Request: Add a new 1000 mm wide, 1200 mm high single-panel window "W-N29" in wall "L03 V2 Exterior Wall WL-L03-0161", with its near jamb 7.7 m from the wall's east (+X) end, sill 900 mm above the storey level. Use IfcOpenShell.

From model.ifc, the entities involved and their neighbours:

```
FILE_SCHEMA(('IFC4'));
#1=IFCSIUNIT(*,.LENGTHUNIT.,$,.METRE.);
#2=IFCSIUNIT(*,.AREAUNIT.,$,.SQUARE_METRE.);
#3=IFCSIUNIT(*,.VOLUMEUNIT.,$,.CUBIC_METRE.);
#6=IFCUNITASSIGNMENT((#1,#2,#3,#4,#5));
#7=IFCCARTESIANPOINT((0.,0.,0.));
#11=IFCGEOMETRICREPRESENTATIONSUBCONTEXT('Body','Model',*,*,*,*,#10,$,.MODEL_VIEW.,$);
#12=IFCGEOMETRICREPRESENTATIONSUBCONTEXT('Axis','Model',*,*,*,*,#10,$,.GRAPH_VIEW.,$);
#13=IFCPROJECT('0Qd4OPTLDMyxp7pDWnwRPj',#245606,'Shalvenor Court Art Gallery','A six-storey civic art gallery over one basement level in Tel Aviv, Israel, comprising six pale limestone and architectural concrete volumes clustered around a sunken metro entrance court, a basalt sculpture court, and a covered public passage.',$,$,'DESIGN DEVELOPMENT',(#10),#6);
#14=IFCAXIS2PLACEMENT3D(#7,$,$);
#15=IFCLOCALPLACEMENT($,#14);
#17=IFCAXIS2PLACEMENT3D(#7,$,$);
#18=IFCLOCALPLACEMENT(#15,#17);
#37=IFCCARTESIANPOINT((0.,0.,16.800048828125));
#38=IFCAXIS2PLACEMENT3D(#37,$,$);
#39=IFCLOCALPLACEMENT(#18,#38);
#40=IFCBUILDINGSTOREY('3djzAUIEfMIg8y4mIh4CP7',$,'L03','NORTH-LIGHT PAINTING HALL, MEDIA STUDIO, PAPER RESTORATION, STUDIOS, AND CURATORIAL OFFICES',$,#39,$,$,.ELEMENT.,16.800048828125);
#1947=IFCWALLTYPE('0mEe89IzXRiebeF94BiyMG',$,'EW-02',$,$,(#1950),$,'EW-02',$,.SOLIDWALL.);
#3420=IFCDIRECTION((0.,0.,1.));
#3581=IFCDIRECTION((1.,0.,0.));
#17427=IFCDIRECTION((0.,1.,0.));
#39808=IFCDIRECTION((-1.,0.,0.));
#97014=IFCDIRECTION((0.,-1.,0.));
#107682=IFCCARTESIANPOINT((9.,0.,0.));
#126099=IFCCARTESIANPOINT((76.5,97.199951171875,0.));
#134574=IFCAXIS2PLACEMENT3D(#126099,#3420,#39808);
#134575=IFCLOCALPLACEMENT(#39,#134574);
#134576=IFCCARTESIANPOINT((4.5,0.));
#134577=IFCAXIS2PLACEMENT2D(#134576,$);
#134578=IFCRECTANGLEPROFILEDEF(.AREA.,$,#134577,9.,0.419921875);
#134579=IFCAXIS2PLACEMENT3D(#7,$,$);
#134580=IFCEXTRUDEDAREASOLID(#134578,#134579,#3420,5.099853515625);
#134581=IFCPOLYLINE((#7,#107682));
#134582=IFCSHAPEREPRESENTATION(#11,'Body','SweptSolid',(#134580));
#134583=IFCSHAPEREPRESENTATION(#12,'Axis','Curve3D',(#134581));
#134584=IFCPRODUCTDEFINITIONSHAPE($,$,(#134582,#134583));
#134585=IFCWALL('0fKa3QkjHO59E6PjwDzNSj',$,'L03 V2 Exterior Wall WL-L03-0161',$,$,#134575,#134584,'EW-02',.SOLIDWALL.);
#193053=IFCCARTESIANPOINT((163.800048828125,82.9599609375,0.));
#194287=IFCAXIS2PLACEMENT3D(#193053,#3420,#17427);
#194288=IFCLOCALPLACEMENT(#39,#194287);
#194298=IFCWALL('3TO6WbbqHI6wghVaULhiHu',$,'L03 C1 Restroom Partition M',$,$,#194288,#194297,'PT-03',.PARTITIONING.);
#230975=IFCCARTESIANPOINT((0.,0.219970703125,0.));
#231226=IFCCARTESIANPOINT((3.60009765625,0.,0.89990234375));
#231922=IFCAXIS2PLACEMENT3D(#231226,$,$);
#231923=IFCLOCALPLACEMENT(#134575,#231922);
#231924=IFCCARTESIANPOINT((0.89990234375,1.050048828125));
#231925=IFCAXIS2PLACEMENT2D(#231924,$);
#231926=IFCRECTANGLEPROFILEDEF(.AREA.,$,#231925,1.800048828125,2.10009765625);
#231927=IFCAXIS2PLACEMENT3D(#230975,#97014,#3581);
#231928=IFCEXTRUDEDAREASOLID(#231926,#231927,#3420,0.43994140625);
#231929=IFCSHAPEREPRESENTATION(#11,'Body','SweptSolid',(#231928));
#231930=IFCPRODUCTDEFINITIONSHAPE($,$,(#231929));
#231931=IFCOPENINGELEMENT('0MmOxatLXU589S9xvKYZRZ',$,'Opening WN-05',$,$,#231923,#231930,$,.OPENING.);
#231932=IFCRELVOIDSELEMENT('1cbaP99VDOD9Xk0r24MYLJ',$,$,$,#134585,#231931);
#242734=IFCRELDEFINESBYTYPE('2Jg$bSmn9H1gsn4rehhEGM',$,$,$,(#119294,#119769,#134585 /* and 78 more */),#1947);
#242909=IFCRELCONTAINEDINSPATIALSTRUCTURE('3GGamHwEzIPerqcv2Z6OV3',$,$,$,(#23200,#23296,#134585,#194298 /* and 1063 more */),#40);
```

```python
import numpy as np
import ifcopenshell
import ifcopenshell.api.feature
import ifcopenshell.api.geometry
import ifcopenshell.api.root
import ifcopenshell.api.spatial
import ifcopenshell.geom
import ifcopenshell.util.element
import ifcopenshell.util.placement
import ifcopenshell.util.representation
import ifcopenshell.util.shape
import ifcopenshell.util.unit

model = ifcopenshell.open("model.ifc")
unit_scale = ifcopenshell.util.unit.calculate_unit_scale(model)
settings = ifcopenshell.geom.settings()


def volume(element):
    """Net volume in cubic metres, openings subtracted."""
    shape = ifcopenshell.geom.create_shape(settings, element)
    return ifcopenshell.util.shape.get_volume(shape.geometry)


wall = model.by_guid("0fKa3QkjHO59E6PjwDzNSj")
storey = ifcopenshell.util.element.get_container(wall, ifc_class="IfcBuildingStorey")
context = ifcopenshell.util.representation.get_context(model, "Model", "Body", "MODEL_VIEW")
before = volume(wall)

width, height, from_end, sill = 1, 1.2, 7.7, 0.9  # metres

# The wall runs along its own X axis, and the end named is its -X end.
wall_shape = ifcopenshell.geom.create_shape(settings, wall)
x, y, z = ifcopenshell.util.shape.get_vertices(wall_shape.geometry).T
start = x.min() + from_end
face, thickness = float(y.min()), float(y.max() - y.min())
wall_matrix = ifcopenshell.util.placement.get_local_placement(wall.ObjectPlacement)
level = ifcopenshell.util.placement.get_local_placement(storey.ObjectPlacement)[2, 3]


def in_wall(x, y):
    """Placement at x, y metres in the wall's axes, at sill height."""
    matrix = wall_matrix.copy()
    matrix[:, 3] = wall_matrix @ np.array([x / unit_scale, y / unit_scale, 0.0, 1.0])
    matrix[2, 3] = level + sill / unit_scale
    return matrix


# Opening: a box that overshoots both wall faces by 50 mm.
opening = ifcopenshell.api.root.create_entity(model, ifc_class="IfcOpeningElement", predefined_type="OPENING")
box = ifcopenshell.api.geometry.add_wall_representation(
    model, context=context, length=width, height=height, thickness=thickness + 0.1
)
ifcopenshell.api.geometry.assign_representation(model, product=opening, representation=box)
ifcopenshell.api.geometry.edit_object_placement(model, product=opening, matrix=in_wall(start, face - 0.05), is_si=False)
ifcopenshell.api.feature.add_feature(model, feature=opening, element=wall)

window = ifcopenshell.api.root.create_entity(model, ifc_class="IfcWindow", name="W-N29", predefined_type="WINDOW")
window.OverallWidth, window.OverallHeight = width / unit_scale, height / unit_scale
window.PartitioningType = "SINGLE_PANEL"
body = ifcopenshell.api.geometry.add_window_representation(
    model,
    context=context,
    overall_width=window.OverallWidth,
    overall_height=window.OverallHeight,
    partition_type="SINGLE_PANEL",
)
ifcopenshell.api.geometry.assign_representation(model, product=window, representation=body)
ifcopenshell.api.spatial.assign_container(model, products=[window], relating_structure=storey)
ifcopenshell.api.feature.add_filling(model, opening=opening, element=window)

# Centre the window in the wall's thickness.
ifcopenshell.api.geometry.edit_object_placement(model, product=window, matrix=in_wall(start, face), is_si=False)
window_shape = ifcopenshell.geom.create_shape(settings, window)
depth = ifcopenshell.util.shape.get_vertices(window_shape.geometry)[:, 1]
offset = face + thickness / 2 - (depth.min() + depth.max()) / 2
ifcopenshell.api.geometry.edit_object_placement(model, product=window, matrix=in_wall(start, offset), is_si=False)

after = volume(wall)

print(f"wall volume {before:.3f} -> {after:.3f} m3")

model.write("model_v2.ifc")
```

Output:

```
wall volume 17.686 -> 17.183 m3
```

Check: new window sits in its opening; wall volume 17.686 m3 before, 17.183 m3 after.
